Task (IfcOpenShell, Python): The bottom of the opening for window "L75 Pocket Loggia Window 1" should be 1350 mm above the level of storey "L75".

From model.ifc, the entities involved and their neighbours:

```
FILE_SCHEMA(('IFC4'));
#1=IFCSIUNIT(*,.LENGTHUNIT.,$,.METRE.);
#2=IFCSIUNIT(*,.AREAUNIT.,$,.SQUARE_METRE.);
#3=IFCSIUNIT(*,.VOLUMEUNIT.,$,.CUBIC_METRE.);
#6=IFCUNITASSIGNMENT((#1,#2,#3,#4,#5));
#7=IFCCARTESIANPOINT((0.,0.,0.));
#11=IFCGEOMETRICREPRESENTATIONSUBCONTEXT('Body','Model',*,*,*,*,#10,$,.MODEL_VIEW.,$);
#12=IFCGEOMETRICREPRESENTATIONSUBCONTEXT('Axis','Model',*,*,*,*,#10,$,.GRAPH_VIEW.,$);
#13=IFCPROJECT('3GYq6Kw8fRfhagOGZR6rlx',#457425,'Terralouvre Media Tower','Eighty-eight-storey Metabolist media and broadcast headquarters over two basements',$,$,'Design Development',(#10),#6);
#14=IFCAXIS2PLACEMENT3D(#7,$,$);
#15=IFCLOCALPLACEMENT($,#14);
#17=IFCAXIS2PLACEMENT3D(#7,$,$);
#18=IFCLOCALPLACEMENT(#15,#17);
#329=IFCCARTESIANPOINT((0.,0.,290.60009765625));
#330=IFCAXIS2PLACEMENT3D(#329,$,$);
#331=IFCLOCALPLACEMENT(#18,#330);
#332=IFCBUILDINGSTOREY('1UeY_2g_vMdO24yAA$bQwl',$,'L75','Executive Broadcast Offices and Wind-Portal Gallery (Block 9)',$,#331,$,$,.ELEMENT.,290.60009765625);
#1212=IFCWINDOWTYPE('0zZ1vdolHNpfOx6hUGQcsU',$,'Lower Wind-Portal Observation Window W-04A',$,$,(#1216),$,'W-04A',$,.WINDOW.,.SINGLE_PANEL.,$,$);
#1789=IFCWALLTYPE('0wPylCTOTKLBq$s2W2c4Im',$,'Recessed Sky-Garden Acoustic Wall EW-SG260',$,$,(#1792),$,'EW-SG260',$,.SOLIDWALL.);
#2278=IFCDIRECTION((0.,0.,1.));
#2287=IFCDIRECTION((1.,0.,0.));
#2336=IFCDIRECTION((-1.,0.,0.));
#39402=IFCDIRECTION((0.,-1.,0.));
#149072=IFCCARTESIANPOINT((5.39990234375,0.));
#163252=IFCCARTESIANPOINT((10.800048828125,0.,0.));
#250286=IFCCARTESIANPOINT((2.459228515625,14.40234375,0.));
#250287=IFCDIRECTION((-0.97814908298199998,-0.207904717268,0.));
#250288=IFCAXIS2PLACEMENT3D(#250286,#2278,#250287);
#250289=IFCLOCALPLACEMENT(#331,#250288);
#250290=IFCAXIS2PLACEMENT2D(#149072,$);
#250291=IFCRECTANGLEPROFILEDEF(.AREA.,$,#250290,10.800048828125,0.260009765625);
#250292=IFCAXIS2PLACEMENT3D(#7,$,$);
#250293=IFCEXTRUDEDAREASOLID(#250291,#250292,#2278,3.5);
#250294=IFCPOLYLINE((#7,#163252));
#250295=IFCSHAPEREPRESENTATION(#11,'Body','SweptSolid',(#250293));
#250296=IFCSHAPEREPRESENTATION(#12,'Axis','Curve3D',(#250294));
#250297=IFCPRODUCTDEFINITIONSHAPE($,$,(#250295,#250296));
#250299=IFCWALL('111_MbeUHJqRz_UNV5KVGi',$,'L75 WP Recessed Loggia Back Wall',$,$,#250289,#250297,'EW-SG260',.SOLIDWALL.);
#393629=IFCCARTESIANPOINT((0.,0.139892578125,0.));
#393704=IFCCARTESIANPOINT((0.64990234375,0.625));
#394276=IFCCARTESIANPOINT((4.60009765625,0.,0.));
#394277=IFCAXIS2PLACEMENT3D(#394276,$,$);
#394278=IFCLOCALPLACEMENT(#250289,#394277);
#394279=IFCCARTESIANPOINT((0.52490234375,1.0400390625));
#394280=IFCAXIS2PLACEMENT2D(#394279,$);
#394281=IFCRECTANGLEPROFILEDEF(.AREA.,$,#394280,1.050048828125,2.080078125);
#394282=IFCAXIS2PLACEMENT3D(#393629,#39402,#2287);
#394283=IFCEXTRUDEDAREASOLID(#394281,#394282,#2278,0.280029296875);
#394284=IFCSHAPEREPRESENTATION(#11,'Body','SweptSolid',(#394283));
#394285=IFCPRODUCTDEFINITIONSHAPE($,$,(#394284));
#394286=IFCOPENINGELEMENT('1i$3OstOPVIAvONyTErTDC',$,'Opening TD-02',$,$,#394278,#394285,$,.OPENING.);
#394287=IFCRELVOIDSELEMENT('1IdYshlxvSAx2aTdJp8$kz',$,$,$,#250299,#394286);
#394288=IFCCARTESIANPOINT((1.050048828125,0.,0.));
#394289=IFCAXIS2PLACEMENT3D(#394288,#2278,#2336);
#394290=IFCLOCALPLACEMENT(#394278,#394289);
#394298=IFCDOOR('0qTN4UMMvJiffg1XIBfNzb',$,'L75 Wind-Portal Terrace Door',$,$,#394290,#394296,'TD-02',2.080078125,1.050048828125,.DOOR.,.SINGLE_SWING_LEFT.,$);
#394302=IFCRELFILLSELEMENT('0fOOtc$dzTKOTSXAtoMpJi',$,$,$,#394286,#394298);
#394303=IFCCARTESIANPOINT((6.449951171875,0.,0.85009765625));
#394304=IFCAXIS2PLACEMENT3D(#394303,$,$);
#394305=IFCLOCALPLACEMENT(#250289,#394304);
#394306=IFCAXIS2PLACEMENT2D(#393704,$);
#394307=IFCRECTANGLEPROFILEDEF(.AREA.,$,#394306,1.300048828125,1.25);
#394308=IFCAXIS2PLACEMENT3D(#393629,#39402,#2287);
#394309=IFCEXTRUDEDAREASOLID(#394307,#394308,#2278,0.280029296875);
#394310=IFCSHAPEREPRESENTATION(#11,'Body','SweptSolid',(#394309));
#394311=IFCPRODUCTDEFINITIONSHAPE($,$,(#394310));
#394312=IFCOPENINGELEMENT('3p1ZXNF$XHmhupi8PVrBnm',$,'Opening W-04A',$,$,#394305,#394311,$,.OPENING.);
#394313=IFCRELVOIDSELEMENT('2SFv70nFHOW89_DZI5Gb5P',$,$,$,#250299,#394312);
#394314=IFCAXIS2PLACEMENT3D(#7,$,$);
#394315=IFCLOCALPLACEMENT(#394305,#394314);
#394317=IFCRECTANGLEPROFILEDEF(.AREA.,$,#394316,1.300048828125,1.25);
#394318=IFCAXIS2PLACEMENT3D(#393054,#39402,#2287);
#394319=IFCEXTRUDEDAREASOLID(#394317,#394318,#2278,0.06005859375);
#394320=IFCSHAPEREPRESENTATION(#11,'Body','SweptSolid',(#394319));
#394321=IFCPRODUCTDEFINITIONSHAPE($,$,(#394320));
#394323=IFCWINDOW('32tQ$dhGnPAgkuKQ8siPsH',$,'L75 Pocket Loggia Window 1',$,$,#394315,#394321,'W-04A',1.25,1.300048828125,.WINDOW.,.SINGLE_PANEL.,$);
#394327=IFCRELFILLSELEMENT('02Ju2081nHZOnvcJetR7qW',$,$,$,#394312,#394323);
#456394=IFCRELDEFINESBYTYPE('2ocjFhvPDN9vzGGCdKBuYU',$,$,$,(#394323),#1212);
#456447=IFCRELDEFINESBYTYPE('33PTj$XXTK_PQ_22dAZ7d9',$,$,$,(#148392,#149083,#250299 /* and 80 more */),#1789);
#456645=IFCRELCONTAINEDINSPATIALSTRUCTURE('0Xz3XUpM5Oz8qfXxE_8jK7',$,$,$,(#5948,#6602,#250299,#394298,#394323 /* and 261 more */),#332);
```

```python
import numpy as np
import ifcopenshell
import ifcopenshell.api.geometry
import ifcopenshell.geom
import ifcopenshell.util.element
import ifcopenshell.util.placement
import ifcopenshell.util.shape
import ifcopenshell.util.unit

model = ifcopenshell.open("model.ifc")
unit_scale = ifcopenshell.util.unit.calculate_unit_scale(model)

window = model.by_guid("32tQ$dhGnPAgkuKQ8siPsH")
opening = window.FillsVoids[0].RelatingOpeningElement
storey = ifcopenshell.util.element.get_container(window, ifc_class="IfcBuildingStorey")
level = ifcopenshell.util.placement.get_local_placement(storey.ObjectPlacement)[2, 3]

# The opening's origin need not be at the sill, so measure its lowest point.
shape = ifcopenshell.geom.create_shape(ifcopenshell.geom.settings(), opening)
bottom = ifcopenshell.util.shape.get_shape_bottom_elevation(shape, shape.geometry) / unit_scale
dz = level + 1.35 / unit_scale - bottom

shift = np.array([0.0, 0.0, dz])
# The window is placed relative to its opening, so it follows when the opening moves.
matrix = ifcopenshell.util.placement.get_local_placement(opening.ObjectPlacement)
matrix[:3, 3] += shift
ifcopenshell.api.geometry.edit_object_placement(
    model, product=opening, matrix=matrix, is_si=False, should_transform_children=True
)

print(f"moved by {dz * unit_scale:+.3f} m")

model.write("model_rev.ifc")
```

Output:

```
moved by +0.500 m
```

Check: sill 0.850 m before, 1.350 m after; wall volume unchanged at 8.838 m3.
